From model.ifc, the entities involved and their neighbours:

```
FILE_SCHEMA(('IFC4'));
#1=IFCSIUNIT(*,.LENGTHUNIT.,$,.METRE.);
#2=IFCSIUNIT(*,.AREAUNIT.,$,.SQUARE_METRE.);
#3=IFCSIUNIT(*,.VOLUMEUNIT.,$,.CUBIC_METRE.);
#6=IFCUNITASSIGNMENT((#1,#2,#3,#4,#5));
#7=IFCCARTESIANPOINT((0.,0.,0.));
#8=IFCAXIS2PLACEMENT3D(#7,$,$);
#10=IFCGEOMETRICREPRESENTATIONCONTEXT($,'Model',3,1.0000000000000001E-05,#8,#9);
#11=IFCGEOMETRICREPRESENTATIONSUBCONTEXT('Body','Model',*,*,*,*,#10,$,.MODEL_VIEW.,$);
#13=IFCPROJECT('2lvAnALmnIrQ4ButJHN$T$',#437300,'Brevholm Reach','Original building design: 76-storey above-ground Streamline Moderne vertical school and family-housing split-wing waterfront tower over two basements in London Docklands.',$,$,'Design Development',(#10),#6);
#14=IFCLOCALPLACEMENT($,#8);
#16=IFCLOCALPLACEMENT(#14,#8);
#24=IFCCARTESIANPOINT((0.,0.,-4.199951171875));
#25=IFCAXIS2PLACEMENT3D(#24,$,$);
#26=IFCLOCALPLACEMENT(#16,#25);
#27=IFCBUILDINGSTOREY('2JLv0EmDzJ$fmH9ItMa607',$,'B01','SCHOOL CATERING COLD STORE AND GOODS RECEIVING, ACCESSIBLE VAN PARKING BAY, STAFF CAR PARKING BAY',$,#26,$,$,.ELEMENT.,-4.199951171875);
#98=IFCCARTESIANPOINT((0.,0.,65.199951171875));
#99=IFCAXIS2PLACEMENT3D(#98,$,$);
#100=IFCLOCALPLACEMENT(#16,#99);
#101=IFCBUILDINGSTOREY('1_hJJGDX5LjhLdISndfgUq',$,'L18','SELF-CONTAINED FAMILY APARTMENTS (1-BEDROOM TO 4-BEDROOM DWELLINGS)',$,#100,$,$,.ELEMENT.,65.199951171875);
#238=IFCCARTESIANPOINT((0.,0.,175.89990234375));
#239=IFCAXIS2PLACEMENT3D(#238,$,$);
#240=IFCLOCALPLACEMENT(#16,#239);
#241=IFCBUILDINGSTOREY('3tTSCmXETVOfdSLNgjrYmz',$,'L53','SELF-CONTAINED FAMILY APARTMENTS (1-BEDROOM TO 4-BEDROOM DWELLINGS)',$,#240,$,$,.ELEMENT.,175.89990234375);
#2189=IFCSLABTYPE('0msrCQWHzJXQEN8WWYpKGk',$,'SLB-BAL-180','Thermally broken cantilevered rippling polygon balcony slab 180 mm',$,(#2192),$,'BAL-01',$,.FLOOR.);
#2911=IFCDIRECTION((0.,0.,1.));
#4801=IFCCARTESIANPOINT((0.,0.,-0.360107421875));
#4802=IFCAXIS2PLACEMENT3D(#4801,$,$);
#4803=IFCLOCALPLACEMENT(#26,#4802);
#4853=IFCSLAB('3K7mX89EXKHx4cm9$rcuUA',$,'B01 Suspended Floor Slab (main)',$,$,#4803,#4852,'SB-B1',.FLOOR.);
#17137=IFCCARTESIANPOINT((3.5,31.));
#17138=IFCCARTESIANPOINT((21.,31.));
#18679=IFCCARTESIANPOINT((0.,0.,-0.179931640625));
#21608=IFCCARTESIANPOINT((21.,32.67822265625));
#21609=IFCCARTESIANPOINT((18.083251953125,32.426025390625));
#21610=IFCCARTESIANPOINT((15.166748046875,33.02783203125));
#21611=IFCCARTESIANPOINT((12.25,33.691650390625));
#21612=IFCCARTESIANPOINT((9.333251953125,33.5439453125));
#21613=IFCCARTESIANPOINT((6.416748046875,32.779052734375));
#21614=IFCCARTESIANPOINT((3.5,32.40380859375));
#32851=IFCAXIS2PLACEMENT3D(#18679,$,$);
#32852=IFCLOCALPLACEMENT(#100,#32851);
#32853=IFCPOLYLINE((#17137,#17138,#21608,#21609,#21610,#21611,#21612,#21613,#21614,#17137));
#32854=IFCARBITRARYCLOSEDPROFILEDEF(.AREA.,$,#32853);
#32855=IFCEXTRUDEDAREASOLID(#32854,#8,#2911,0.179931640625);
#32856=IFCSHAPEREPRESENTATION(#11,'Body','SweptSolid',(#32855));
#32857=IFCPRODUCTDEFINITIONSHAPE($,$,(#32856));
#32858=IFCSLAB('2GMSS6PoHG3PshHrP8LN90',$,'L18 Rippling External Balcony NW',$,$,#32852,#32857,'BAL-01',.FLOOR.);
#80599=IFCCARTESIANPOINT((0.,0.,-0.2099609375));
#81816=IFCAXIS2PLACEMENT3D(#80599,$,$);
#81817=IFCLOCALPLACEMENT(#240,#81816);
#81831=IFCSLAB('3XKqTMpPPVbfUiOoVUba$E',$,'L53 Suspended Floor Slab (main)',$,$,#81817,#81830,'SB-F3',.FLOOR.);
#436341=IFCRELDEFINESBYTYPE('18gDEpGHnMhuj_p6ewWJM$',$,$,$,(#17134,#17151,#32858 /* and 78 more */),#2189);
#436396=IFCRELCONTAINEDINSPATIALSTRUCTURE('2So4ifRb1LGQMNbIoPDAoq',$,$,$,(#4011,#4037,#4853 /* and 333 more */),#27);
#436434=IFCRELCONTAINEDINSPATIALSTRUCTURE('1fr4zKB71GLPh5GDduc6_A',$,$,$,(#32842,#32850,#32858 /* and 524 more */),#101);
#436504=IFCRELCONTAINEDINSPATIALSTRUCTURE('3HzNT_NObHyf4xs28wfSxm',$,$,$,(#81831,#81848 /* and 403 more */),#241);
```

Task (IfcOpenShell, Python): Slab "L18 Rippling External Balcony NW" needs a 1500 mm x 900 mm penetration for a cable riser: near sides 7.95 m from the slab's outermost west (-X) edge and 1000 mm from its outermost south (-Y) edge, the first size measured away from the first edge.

```python
import numpy as np
import ifcopenshell
import ifcopenshell.api.feature
import ifcopenshell.api.geometry
import ifcopenshell.api.root
import ifcopenshell.geom
import ifcopenshell.util.placement
import ifcopenshell.util.representation
import ifcopenshell.util.shape
import ifcopenshell.util.unit

model = ifcopenshell.open("model.ifc")
unit_scale = ifcopenshell.util.unit.calculate_unit_scale(model)
settings = ifcopenshell.geom.settings()


def volume(element):
    """Net volume in cubic metres, openings subtracted."""
    shape = ifcopenshell.geom.create_shape(settings, element)
    return ifcopenshell.util.shape.get_volume(shape.geometry)


slab = model.by_guid("2GMSS6PoHG3PshHrP8LN90")
before = volume(slab)

# Extent in the slab's own axes, in metres. The edges named are its -X and -Y sides.
slab_shape = ifcopenshell.geom.create_shape(settings, slab)
vertices = ifcopenshell.util.shape.get_vertices(slab_shape.geometry)
x_min, y_min, bottom = vertices.min(axis=0)
top = vertices[:, 2].max()

opening = ifcopenshell.api.root.create_entity(model, ifc_class="IfcOpeningElement", name="Cable riser opening", predefined_type="OPENING")
context = ifcopenshell.util.representation.get_context(model, "Model", "Body", "MODEL_VIEW")
width, depth = 1.5, 0.9
outline = [(0.0, 0.0), (width, 0.0), (width, depth), (0.0, depth), (0.0, 0.0)]
# Overshoot both faces by 50 mm so the cut is clean.
shape = ifcopenshell.api.geometry.add_slab_representation(
    model, context=context, depth=top - bottom + 0.1, polyline=outline
)
ifcopenshell.api.geometry.assign_representation(model, product=opening, representation=shape)

matrix = ifcopenshell.util.placement.get_local_placement(slab.ObjectPlacement)
matrix[:, 3] = matrix @ np.append(np.array([x_min + 7.95, y_min + 1, bottom - 0.05]) / unit_scale, 1.0)
ifcopenshell.api.geometry.edit_object_placement(model, product=opening, matrix=matrix, is_si=False)
ifcopenshell.api.feature.add_feature(model, feature=opening, element=slab)

after = volume(slab)

print(f"slab volume {before:.3f} -> {after:.3f} m3")

model.write("model_v2.ifc")
```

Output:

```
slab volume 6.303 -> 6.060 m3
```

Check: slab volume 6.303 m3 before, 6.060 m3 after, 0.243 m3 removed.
